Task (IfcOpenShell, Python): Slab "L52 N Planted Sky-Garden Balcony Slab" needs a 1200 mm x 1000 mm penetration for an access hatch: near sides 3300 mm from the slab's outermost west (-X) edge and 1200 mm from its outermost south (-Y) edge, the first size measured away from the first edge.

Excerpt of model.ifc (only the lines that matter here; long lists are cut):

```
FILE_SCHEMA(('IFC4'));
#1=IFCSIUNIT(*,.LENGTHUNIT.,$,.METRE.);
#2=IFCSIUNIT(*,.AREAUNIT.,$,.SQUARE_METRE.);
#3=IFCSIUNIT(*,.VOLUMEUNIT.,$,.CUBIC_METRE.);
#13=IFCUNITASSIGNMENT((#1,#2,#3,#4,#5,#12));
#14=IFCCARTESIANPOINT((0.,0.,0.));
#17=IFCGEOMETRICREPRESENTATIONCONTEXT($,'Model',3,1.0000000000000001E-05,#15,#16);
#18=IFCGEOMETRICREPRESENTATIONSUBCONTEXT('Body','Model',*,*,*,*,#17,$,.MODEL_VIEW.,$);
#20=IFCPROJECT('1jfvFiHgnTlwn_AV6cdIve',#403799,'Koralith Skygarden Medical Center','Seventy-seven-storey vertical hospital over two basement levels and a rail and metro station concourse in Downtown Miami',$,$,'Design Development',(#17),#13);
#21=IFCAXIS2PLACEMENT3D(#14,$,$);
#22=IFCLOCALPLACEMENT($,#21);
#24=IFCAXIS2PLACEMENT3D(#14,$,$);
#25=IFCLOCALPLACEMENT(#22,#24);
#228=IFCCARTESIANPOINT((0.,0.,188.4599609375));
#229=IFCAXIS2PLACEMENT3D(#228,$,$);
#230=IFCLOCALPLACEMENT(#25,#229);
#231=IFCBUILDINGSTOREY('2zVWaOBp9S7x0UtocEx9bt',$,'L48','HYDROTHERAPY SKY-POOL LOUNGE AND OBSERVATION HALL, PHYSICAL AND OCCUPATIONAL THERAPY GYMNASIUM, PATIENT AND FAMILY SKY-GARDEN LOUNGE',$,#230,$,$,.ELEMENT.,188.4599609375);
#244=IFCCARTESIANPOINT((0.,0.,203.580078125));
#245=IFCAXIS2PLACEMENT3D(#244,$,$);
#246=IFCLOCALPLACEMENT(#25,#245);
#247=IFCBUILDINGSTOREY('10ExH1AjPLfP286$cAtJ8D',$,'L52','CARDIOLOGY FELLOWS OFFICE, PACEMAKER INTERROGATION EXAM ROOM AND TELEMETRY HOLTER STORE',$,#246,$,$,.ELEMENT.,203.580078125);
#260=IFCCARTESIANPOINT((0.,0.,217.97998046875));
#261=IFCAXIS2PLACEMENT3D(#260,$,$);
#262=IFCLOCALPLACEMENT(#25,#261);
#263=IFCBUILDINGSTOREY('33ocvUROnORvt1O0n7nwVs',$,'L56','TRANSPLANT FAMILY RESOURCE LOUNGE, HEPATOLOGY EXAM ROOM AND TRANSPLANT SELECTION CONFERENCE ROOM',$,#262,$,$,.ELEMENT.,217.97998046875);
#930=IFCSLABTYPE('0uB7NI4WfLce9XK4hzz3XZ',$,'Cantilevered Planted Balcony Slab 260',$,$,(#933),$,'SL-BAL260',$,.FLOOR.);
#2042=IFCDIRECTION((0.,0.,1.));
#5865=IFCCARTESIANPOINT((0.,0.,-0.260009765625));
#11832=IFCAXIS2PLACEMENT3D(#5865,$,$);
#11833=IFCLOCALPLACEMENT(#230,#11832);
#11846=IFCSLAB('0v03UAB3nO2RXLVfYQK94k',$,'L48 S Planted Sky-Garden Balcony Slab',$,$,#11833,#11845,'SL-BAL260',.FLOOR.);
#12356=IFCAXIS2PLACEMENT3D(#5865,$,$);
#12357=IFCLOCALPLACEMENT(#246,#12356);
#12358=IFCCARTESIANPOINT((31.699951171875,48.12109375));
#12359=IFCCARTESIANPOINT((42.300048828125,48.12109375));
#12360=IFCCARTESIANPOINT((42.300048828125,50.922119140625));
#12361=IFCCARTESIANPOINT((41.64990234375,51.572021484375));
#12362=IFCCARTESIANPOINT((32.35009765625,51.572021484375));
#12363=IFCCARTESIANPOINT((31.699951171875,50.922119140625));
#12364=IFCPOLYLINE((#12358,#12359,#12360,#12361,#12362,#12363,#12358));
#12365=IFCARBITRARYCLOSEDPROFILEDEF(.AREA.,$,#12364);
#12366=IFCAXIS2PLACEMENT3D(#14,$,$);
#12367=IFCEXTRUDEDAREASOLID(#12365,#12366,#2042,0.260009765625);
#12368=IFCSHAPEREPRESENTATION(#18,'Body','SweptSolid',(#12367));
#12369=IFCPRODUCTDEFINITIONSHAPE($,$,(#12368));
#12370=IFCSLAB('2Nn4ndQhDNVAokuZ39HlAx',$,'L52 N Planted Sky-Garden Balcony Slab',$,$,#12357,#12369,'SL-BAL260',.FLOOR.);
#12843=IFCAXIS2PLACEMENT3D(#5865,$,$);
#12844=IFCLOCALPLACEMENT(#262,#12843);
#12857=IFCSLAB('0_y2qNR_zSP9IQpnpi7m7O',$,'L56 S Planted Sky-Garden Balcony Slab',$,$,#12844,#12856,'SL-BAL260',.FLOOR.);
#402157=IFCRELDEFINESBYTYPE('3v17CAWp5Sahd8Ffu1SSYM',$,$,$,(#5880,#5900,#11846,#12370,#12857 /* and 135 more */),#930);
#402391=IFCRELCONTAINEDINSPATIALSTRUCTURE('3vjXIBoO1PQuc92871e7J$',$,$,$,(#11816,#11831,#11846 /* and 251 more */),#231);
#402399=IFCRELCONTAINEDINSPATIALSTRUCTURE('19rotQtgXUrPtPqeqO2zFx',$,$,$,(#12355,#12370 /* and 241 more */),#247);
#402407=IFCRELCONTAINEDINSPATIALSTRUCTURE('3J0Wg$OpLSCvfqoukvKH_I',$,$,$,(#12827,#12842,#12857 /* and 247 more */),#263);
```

```python
import numpy as np
import ifcopenshell
import ifcopenshell.api.feature
import ifcopenshell.api.geometry
import ifcopenshell.api.root
import ifcopenshell.geom
import ifcopenshell.util.placement
import ifcopenshell.util.representation
import ifcopenshell.util.shape
import ifcopenshell.util.unit

model = ifcopenshell.open("model.ifc")
unit_scale = ifcopenshell.util.unit.calculate_unit_scale(model)
settings = ifcopenshell.geom.settings()


def volume(element):
    """Net volume in cubic metres, openings subtracted."""
    shape = ifcopenshell.geom.create_shape(settings, element)
    return ifcopenshell.util.shape.get_volume(shape.geometry)


slab = model.by_guid("2Nn4ndQhDNVAokuZ39HlAx")
before = volume(slab)

# Extent in the slab's own axes, in metres. The edges named are its -X and -Y sides.
slab_shape = ifcopenshell.geom.create_shape(settings, slab)
vertices = ifcopenshell.util.shape.get_vertices(slab_shape.geometry)
x_min, y_min, bottom = vertices.min(axis=0)
top = vertices[:, 2].max()

opening = ifcopenshell.api.root.create_entity(model, ifc_class="IfcOpeningElement", name="Access hatch opening", predefined_type="OPENING")
context = ifcopenshell.util.representation.get_context(model, "Model", "Body", "MODEL_VIEW")
width, depth = 1.2, 1
outline = [(0.0, 0.0), (width, 0.0), (width, depth), (0.0, depth), (0.0, 0.0)]
# Overshoot both faces by 50 mm so the cut is clean.
shape = ifcopenshell.api.geometry.add_slab_representation(
    model, context=context, depth=top - bottom + 0.1, polyline=outline
)
ifcopenshell.api.geometry.assign_representation(model, product=opening, representation=shape)

matrix = ifcopenshell.util.placement.get_local_placement(slab.ObjectPlacement)
matrix[:, 3] = matrix @ np.append(np.array([x_min + 3.3, y_min + 1.2, bottom - 0.05]) / unit_scale, 1.0)
ifcopenshell.api.geometry.edit_object_placement(model, product=opening, matrix=matrix, is_si=False)
ifcopenshell.api.feature.add_feature(model, feature=opening, element=slab)

after = volume(slab)

print(f"slab volume {before:.3f} -> {after:.3f} m3")

model.write("model_v2.ifc")
```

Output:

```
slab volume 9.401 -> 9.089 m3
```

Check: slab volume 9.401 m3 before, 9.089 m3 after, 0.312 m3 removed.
